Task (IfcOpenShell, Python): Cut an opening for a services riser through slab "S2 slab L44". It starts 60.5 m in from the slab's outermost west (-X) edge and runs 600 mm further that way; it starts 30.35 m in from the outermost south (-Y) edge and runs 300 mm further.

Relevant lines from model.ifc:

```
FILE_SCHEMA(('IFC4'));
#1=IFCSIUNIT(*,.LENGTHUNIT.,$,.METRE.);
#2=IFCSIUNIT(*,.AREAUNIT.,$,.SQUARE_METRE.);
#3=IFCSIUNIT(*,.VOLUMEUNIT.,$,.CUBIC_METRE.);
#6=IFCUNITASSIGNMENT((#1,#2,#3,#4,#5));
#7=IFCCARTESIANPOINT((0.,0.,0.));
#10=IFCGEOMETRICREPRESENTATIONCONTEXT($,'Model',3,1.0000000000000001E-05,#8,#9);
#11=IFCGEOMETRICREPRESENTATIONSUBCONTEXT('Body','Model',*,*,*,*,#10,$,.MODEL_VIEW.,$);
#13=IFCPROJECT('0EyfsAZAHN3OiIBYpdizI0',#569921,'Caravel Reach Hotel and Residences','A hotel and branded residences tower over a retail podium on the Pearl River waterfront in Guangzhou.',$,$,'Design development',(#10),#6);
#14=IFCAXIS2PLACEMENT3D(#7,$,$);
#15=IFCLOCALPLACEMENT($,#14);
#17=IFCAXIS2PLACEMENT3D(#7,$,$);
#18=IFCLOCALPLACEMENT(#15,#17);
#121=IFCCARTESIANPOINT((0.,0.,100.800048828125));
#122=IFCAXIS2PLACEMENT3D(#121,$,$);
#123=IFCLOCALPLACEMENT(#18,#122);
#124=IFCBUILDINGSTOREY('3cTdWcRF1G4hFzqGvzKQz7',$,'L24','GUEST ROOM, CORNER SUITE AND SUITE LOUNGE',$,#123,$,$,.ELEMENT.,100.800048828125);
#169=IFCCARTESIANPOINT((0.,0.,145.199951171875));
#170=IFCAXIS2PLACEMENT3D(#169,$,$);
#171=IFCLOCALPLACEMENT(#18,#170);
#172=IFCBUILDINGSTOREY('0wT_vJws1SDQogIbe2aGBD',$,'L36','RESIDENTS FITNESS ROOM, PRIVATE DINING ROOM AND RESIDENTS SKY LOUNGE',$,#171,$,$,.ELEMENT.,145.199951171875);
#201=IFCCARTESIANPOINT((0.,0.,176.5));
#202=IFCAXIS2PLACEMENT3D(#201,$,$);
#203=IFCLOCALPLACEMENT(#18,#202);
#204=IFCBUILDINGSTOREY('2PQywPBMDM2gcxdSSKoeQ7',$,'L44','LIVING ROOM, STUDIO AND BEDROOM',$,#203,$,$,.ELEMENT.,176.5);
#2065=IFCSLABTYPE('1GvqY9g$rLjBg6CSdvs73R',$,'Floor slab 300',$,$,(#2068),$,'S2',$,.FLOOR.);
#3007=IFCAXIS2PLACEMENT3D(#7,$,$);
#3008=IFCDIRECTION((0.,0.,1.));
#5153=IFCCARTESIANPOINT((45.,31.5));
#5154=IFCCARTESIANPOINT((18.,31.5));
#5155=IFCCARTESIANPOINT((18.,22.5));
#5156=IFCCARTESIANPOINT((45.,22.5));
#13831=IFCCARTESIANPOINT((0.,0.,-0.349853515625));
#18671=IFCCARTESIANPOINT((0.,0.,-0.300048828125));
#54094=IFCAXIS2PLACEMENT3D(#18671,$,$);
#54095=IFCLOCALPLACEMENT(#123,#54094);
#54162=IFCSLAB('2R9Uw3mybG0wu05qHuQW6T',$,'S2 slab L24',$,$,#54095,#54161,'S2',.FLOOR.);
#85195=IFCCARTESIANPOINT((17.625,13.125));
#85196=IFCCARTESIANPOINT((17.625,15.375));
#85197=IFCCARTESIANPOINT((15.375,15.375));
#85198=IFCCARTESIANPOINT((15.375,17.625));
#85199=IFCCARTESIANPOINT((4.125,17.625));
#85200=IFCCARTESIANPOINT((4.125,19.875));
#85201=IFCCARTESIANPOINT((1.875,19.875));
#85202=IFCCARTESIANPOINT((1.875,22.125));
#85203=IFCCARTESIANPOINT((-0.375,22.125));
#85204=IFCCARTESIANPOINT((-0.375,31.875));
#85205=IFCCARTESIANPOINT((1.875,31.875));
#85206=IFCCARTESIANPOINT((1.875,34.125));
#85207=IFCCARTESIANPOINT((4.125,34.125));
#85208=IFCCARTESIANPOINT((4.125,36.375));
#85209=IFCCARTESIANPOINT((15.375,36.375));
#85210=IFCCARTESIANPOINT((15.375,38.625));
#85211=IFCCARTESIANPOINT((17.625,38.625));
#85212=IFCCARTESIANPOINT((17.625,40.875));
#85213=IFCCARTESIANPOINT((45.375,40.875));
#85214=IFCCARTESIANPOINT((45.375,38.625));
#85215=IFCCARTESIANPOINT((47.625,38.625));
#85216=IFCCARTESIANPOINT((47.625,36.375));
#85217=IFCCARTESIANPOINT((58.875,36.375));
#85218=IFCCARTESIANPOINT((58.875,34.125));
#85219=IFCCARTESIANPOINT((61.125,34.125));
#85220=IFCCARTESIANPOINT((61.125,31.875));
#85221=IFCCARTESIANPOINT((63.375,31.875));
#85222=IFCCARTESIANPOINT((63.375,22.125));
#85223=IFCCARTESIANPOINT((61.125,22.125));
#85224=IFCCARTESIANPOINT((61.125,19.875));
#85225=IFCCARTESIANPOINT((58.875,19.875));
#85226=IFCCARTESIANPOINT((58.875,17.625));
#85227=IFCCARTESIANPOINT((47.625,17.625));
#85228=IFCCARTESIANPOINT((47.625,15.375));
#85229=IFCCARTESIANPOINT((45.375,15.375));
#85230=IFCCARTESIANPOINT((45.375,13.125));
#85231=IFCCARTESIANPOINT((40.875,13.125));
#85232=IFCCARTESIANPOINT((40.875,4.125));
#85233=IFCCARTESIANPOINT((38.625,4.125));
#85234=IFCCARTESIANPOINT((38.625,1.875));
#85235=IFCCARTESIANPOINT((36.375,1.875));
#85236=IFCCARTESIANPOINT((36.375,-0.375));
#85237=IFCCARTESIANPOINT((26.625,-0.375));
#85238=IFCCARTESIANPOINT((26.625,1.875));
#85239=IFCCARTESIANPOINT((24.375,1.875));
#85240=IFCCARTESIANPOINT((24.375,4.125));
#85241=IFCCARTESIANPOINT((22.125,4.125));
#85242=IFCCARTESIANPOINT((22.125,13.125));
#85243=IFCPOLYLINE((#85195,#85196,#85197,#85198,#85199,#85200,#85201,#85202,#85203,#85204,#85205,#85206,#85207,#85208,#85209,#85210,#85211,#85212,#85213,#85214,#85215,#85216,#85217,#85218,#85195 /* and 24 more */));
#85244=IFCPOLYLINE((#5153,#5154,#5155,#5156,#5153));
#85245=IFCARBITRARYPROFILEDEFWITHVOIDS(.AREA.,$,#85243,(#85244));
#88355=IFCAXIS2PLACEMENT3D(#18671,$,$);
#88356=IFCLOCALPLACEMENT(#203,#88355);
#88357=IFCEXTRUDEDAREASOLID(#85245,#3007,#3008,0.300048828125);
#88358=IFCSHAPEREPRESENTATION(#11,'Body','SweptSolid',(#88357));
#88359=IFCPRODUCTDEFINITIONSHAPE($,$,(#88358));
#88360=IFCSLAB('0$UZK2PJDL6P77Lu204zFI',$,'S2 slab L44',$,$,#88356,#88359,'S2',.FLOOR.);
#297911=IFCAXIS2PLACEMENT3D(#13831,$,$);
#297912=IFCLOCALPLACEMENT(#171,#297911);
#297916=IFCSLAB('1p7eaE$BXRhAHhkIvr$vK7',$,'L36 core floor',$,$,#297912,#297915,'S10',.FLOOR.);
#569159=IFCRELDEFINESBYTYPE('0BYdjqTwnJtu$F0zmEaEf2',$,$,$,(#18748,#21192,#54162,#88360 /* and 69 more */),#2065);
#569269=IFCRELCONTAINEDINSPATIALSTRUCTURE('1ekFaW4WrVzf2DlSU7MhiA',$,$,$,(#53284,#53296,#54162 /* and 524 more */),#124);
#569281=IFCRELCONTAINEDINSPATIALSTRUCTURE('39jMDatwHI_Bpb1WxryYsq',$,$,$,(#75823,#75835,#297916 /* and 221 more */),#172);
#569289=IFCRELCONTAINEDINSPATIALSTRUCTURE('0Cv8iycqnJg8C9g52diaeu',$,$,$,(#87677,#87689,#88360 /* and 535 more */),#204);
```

```python
import numpy as np
import ifcopenshell
import ifcopenshell.api.feature
import ifcopenshell.api.geometry
import ifcopenshell.api.root
import ifcopenshell.geom
import ifcopenshell.util.placement
import ifcopenshell.util.representation
import ifcopenshell.util.shape
import ifcopenshell.util.unit

model = ifcopenshell.open("model.ifc")
unit_scale = ifcopenshell.util.unit.calculate_unit_scale(model)
settings = ifcopenshell.geom.settings()


def volume(element):
    """Net volume in cubic metres, openings subtracted."""
    shape = ifcopenshell.geom.create_shape(settings, element)
    return ifcopenshell.util.shape.get_volume(shape.geometry)


slab = model.by_id(88360)
before = volume(slab)

# Extent in the slab's own axes, in metres. The edges named are its -X and -Y sides.
slab_shape = ifcopenshell.geom.create_shape(settings, slab)
vertices = ifcopenshell.util.shape.get_vertices(slab_shape.geometry)
x_min, y_min, bottom = vertices.min(axis=0)
top = vertices[:, 2].max()

opening = ifcopenshell.api.root.create_entity(model, ifc_class="IfcOpeningElement", name="Services riser opening", predefined_type="OPENING")
context = ifcopenshell.util.representation.get_context(model, "Model", "Body", "MODEL_VIEW")
width, depth = 0.6, 0.3
outline = [(0.0, 0.0), (width, 0.0), (width, depth), (0.0, depth), (0.0, 0.0)]
# Overshoot both faces by 50 mm so the cut is clean.
shape = ifcopenshell.api.geometry.add_slab_representation(
    model, context=context, depth=top - bottom + 0.1, polyline=outline
)
ifcopenshell.api.geometry.assign_representation(model, product=opening, representation=shape)

matrix = ifcopenshell.util.placement.get_local_placement(slab.ObjectPlacement)
matrix[:, 3] = matrix @ np.append(np.array([x_min + 60.5, y_min + 30.35, bottom - 0.05]) / unit_scale, 1.0)
ifcopenshell.api.geometry.edit_object_placement(model, product=opening, matrix=matrix, is_si=False)
ifcopenshell.api.feature.add_feature(model, feature=opening, element=slab)

after = volume(slab)

print(f"slab volume {before:.3f} -> {after:.3f} m3")

model.write("model_v2.ifc")
```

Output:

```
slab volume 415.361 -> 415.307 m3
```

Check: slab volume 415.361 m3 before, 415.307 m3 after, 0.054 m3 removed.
